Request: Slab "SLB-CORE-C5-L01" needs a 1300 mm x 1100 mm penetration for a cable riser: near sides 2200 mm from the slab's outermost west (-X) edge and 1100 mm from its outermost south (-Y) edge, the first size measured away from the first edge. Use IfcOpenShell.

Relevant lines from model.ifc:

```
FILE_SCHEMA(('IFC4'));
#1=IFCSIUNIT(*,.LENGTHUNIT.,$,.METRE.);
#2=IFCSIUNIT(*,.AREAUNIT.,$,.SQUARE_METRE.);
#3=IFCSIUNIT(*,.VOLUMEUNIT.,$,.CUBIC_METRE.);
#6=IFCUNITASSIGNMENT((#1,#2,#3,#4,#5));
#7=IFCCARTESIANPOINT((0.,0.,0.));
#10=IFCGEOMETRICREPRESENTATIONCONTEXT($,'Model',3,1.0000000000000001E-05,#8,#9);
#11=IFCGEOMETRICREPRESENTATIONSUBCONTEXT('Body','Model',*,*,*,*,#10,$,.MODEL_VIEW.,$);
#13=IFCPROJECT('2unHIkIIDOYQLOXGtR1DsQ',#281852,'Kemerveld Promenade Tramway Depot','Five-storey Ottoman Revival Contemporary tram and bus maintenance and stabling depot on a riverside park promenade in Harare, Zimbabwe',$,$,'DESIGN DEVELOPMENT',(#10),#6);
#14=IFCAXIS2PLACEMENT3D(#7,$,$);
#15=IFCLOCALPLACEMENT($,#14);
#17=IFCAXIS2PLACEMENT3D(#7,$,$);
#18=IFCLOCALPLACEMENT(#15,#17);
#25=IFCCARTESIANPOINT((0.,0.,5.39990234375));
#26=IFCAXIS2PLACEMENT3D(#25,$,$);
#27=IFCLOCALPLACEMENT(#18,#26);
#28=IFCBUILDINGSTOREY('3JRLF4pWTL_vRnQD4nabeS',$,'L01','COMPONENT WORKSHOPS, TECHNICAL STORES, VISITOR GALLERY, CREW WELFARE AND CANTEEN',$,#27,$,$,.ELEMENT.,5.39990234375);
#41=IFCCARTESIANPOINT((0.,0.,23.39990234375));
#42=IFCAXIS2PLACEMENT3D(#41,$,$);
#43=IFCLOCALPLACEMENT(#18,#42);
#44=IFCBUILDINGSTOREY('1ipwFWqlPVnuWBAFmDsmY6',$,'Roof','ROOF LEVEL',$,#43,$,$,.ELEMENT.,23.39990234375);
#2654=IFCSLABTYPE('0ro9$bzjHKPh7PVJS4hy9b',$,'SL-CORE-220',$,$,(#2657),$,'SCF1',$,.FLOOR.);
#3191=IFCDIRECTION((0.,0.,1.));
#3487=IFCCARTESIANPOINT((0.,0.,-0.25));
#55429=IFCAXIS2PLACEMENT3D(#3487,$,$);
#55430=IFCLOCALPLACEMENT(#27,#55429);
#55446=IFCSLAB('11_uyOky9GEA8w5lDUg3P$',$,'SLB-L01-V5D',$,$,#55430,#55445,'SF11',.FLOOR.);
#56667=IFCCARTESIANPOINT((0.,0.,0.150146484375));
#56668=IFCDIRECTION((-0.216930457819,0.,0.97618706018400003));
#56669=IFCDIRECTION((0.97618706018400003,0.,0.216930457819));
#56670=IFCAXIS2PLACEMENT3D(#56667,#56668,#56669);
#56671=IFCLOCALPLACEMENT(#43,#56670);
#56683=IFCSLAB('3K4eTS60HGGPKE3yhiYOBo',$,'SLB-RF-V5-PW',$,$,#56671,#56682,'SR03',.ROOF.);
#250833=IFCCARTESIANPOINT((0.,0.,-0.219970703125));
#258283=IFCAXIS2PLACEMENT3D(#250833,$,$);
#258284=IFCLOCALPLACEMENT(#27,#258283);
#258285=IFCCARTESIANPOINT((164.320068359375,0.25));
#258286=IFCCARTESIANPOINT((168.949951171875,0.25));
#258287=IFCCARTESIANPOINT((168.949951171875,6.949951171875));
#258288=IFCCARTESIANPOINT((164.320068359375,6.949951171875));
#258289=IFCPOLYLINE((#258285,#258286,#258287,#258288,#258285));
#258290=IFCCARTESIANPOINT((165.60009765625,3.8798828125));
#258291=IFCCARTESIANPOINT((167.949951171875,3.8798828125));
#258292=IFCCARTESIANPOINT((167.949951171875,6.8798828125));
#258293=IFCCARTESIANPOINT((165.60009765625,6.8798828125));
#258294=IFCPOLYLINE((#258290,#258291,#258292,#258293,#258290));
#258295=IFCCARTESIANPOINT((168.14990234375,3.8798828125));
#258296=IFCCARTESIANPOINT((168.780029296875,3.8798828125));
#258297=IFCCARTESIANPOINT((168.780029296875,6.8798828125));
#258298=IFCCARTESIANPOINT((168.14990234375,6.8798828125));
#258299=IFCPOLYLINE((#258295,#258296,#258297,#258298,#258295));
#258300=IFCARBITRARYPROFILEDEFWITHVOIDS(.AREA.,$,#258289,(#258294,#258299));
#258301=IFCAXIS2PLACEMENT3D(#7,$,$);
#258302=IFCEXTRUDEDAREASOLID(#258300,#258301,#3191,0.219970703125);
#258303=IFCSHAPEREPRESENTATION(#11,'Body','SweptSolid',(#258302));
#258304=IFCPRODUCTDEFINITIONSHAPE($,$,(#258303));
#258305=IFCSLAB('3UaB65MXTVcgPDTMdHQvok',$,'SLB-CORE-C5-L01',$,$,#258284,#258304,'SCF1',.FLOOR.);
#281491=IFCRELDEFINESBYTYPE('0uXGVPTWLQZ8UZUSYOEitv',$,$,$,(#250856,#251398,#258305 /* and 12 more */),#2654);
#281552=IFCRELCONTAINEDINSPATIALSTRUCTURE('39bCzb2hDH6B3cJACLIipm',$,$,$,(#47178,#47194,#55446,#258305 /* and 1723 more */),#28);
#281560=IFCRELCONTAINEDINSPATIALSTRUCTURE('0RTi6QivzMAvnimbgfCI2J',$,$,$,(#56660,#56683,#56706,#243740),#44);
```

```python
import numpy as np
import ifcopenshell
import ifcopenshell.api.feature
import ifcopenshell.api.geometry
import ifcopenshell.api.root
import ifcopenshell.geom
import ifcopenshell.util.placement
import ifcopenshell.util.representation
import ifcopenshell.util.shape
import ifcopenshell.util.unit

model = ifcopenshell.open("model.ifc")
unit_scale = ifcopenshell.util.unit.calculate_unit_scale(model)
settings = ifcopenshell.geom.settings()


def volume(element):
    """Net volume in cubic metres, openings subtracted."""
    shape = ifcopenshell.geom.create_shape(settings, element)
    return ifcopenshell.util.shape.get_volume(shape.geometry)


slab = model.by_guid("3UaB65MXTVcgPDTMdHQvok")
before = volume(slab)

# Extent in the slab's own axes, in metres. The edges named are its -X and -Y sides.
slab_shape = ifcopenshell.geom.create_shape(settings, slab)
vertices = ifcopenshell.util.shape.get_vertices(slab_shape.geometry)
x_min, y_min, bottom = vertices.min(axis=0)
top = vertices[:, 2].max()

opening = ifcopenshell.api.root.create_entity(model, ifc_class="IfcOpeningElement", name="Cable riser opening", predefined_type="OPENING")
context = ifcopenshell.util.representation.get_context(model, "Model", "Body", "MODEL_VIEW")
width, depth = 1.3, 1.1
outline = [(0.0, 0.0), (width, 0.0), (width, depth), (0.0, depth), (0.0, 0.0)]
# Overshoot both faces by 50 mm so the cut is clean.
shape = ifcopenshell.api.geometry.add_slab_representation(
    model, context=context, depth=top - bottom + 0.1, polyline=outline
)
ifcopenshell.api.geometry.assign_representation(model, product=opening, representation=shape)

matrix = ifcopenshell.util.placement.get_local_placement(slab.ObjectPlacement)
matrix[:, 3] = matrix @ np.append(np.array([x_min + 2.2, y_min + 1.1, bottom - 0.05]) / unit_scale, 1.0)
ifcopenshell.api.geometry.edit_object_placement(model, product=opening, matrix=matrix, is_si=False)
ifcopenshell.api.feature.add_feature(model, feature=opening, element=slab)

after = volume(slab)

print(f"slab volume {before:.3f} -> {after:.3f} m3")

model.write("model_v2.ifc")
```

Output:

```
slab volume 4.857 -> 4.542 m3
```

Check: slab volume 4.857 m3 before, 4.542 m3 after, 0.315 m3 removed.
